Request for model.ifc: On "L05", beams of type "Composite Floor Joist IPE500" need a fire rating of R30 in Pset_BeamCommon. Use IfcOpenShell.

First a look at what the model holds.

```python
import ifcopenshell
import ifcopenshell.util.element

model = ifcopenshell.open("model.ifc")
print(model.schema)
storey = next(s for s in model.by_type("IfcBuildingStorey") if s.Name == "L05")
beams = [e for e in ifcopenshell.util.element.get_decomposition(storey) if e.is_a("IfcBeam")]
seen = {}
for e in beams:
    element_type = ifcopenshell.util.element.get_type(e)
    key = (element_type.Name if element_type != e and element_type else None, ifcopenshell.util.element.get_pset(e, "Pset_BeamCommon", "FireRating"))
    seen[key] = seen.get(key, 0) + 1
for (name, value), count in sorted(seen.items(), key=str):
    print(count, "x", name, "|", value)
```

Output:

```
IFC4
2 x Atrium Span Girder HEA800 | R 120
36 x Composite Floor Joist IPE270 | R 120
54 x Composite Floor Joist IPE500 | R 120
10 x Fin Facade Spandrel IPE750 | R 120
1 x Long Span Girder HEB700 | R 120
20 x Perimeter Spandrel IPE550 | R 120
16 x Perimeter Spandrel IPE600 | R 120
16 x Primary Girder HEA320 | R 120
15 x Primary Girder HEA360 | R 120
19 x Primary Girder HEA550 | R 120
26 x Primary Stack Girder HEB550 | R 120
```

```python
import ifcopenshell
import ifcopenshell.api.pset
import ifcopenshell.util.element

model = ifcopenshell.open("model.ifc")

storey = next(s for s in model.by_type("IfcBuildingStorey") if s.Name == "L05")
beams = [e for e in ifcopenshell.util.element.get_decomposition(storey) if e.is_a("IfcBeam")]

count = 0
for e in beams:
    element_type = ifcopenshell.util.element.get_type(e)
    if element_type in (None, e) or element_type.Name != "Composite Floor Joist IPE500":
        continue
    # add_pset returns the element's existing set when there is one.
    pset = ifcopenshell.api.pset.add_pset(model, product=e, name="Pset_BeamCommon")
    ifcopenshell.api.pset.edit_pset(model, pset=pset, properties={"FireRating": "R30"})
    count += 1

print(count, "beams updated")

model.write("model_rev.ifc")
```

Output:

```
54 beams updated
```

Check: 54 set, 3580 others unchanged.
